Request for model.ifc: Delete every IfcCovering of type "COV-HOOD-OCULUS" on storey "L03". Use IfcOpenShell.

First a look at what the model holds.

```python
import ifcopenshell
import ifcopenshell.util.element

model = ifcopenshell.open("model.ifc")
print(model.schema)
storey = next(s for s in model.by_type("IfcBuildingStorey") if s.Name == "L03")
coverings = [e for e in ifcopenshell.util.element.get_decomposition(storey) if e.is_a("IfcCovering")]
seen = {}
for e in coverings:
    element_type = ifcopenshell.util.element.get_type(e)
    name = element_type.Name if element_type not in (None, e) else None
    seen[name] = seen.get(name, 0) + 1
for name, count in sorted(seen.items(), key=str):
    print(count, "x", name)
```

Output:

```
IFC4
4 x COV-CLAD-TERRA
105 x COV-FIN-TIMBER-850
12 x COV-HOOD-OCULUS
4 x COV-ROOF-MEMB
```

```python
import ifcopenshell
import ifcopenshell.api.root
import ifcopenshell.util.element

model = ifcopenshell.open("model.ifc")

storey = next(s for s in model.by_type("IfcBuildingStorey") if s.Name == "L03")
coverings = [e for e in ifcopenshell.util.element.get_decomposition(storey) if e.is_a("IfcCovering")]
targets = [e for e in coverings if (t := ifcopenshell.util.element.get_type(e)) not in (None, e) and t.Name == "COV-HOOD-OCULUS"]

for e in targets:
    ifcopenshell.api.root.remove_product(model, product=e)
print(len(targets), "removed")

model.write("model-out.ifc")
```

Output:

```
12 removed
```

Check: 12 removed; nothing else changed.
